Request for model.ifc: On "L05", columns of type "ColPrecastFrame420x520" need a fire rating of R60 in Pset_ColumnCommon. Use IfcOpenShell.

First a look at what the model holds.

```python
import ifcopenshell
import ifcopenshell.util.element

model = ifcopenshell.open("model.ifc")
print(model.schema)
storey = next(s for s in model.by_type("IfcBuildingStorey") if s.Name == "L05")
columns = [e for e in ifcopenshell.util.element.get_decomposition(storey) if e.is_a("IfcColumn")]
seen = {}
for e in columns:
    element_type = ifcopenshell.util.element.get_type(e)
    key = (element_type.Name if element_type != e and element_type else None, ifcopenshell.util.element.get_pset(e, "Pset_ColumnCommon", "FireRating"))
    seen[key] = seen.get(key, 0) + 1
for (name, value), count in sorted(seen.items(), key=str):
    print(count, "x", name, "|", value)
```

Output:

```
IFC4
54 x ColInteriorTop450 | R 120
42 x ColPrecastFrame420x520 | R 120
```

```python
import ifcopenshell
import ifcopenshell.api.pset
import ifcopenshell.util.element

model = ifcopenshell.open("model.ifc")

storey = next(s for s in model.by_type("IfcBuildingStorey") if s.Name == "L05")
columns = [e for e in ifcopenshell.util.element.get_decomposition(storey) if e.is_a("IfcColumn")]

count = 0
for e in columns:
    element_type = ifcopenshell.util.element.get_type(e)
    if element_type in (None, e) or element_type.Name != "ColPrecastFrame420x520":
        continue
    # add_pset returns the element's existing set when there is one.
    pset = ifcopenshell.api.pset.add_pset(model, product=e, name="Pset_ColumnCommon")
    ifcopenshell.api.pset.edit_pset(model, pset=pset, properties={"FireRating": "R60"})
    count += 1

print(count, "columns updated")

model.write("model_edited.ifc")
```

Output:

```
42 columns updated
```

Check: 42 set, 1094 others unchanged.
